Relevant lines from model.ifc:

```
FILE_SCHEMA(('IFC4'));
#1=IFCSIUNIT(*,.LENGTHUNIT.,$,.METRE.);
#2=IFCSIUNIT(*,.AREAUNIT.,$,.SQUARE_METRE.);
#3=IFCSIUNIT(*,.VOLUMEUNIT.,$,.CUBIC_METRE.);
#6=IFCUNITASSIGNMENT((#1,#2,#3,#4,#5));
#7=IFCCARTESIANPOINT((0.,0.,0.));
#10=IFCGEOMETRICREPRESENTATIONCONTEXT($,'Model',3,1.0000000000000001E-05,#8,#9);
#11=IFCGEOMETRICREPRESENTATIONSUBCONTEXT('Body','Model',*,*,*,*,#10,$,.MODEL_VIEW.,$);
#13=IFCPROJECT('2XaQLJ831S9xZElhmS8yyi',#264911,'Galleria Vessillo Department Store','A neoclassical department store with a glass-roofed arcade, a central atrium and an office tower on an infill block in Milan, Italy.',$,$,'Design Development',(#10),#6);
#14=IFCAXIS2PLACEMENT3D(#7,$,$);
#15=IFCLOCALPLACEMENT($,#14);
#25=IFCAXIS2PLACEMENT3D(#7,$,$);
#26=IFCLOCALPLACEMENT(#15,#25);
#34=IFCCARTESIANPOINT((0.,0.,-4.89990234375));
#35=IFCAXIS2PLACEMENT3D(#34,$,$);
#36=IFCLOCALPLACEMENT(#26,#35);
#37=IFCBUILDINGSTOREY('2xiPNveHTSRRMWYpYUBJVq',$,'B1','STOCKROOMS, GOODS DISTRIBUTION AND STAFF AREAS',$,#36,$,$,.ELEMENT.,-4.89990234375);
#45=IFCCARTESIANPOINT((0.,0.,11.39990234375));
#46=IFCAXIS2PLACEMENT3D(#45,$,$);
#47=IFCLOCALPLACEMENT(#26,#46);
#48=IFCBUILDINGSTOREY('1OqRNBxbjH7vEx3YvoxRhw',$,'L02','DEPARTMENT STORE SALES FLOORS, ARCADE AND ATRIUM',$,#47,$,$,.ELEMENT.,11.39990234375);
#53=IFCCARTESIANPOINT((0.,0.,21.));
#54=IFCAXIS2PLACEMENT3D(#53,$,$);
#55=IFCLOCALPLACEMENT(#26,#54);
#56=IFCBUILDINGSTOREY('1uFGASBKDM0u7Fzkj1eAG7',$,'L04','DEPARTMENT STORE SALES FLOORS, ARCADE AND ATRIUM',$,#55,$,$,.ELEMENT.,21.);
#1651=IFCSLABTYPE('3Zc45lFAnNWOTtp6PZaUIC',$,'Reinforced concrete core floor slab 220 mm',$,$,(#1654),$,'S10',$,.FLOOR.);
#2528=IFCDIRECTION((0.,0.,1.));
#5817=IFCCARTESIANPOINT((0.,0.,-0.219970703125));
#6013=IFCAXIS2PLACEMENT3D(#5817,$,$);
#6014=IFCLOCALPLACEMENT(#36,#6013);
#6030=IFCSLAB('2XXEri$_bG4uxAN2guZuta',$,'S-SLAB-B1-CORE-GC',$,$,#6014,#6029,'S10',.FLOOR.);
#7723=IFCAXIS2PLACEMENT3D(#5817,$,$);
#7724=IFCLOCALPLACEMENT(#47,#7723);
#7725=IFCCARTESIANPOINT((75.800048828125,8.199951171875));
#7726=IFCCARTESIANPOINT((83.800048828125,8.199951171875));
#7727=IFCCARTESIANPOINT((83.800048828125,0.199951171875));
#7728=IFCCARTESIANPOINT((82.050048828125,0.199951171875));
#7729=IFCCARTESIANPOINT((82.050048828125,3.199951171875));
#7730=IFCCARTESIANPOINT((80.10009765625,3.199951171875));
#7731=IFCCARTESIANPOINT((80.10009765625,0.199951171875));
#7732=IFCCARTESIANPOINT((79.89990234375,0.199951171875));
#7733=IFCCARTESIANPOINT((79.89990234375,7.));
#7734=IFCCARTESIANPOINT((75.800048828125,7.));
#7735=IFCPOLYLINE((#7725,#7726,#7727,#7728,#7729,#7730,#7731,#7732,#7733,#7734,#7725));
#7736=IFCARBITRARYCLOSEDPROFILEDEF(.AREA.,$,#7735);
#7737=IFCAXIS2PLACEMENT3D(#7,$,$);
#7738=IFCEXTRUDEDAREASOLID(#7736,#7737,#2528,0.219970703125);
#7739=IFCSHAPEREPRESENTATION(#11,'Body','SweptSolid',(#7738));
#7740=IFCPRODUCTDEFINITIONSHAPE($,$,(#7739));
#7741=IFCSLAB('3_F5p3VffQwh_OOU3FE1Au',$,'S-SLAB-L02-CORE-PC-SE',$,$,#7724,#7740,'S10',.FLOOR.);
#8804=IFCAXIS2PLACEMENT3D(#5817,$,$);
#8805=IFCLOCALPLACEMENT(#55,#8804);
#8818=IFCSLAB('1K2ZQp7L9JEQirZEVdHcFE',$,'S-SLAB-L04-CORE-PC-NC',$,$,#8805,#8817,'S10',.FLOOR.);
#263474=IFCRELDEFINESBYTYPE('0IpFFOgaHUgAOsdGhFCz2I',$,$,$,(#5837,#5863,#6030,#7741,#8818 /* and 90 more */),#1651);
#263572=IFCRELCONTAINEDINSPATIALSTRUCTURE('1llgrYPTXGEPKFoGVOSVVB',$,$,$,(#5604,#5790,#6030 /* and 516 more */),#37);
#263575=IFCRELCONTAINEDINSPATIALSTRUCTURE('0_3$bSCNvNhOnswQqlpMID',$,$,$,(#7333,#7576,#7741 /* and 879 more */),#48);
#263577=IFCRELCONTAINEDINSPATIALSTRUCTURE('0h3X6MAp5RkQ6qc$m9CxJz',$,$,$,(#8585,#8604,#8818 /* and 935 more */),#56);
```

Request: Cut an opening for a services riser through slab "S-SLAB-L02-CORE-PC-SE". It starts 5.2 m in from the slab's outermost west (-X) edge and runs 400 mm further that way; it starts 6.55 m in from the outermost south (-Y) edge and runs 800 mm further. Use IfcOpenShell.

```python
import numpy as np
import ifcopenshell
import ifcopenshell.api.feature
import ifcopenshell.api.geometry
import ifcopenshell.api.root
import ifcopenshell.geom
import ifcopenshell.util.placement
import ifcopenshell.util.representation
import ifcopenshell.util.shape
import ifcopenshell.util.unit

model = ifcopenshell.open("model.ifc")
unit_scale = ifcopenshell.util.unit.calculate_unit_scale(model)
settings = ifcopenshell.geom.settings()


def volume(element):
    """Net volume in cubic metres, openings subtracted."""
    shape = ifcopenshell.geom.create_shape(settings, element)
    return ifcopenshell.util.shape.get_volume(shape.geometry)


slab = model.by_guid("3_F5p3VffQwh_OOU3FE1Au")
before = volume(slab)

# Extent in the slab's own axes, in metres. The edges named are its -X and -Y sides.
slab_shape = ifcopenshell.geom.create_shape(settings, slab)
vertices = ifcopenshell.util.shape.get_vertices(slab_shape.geometry)
x_min, y_min, bottom = vertices.min(axis=0)
top = vertices[:, 2].max()

opening = ifcopenshell.api.root.create_entity(model, ifc_class="IfcOpeningElement", name="Services riser opening", predefined_type="OPENING")
context = ifcopenshell.util.representation.get_context(model, "Model", "Body", "MODEL_VIEW")
width, depth = 0.4, 0.8
outline = [(0.0, 0.0), (width, 0.0), (width, depth), (0.0, depth), (0.0, 0.0)]
# Overshoot both faces by 50 mm so the cut is clean.
shape = ifcopenshell.api.geometry.add_slab_representation(
    model, context=context, depth=top - bottom + 0.1, polyline=outline
)
ifcopenshell.api.geometry.assign_representation(model, product=opening, representation=shape)

matrix = ifcopenshell.util.placement.get_local_placement(slab.ObjectPlacement)
matrix[:, 3] = matrix @ np.append(np.array([x_min + 5.2, y_min + 6.55, bottom - 0.05]) / unit_scale, 1.0)
ifcopenshell.api.geometry.edit_object_placement(model, product=opening, matrix=matrix, is_si=False)
ifcopenshell.api.feature.add_feature(model, feature=opening, element=slab)

after = volume(slab)

print(f"slab volume {before:.3f} -> {after:.3f} m3")

model.write("model_rev.ifc")
```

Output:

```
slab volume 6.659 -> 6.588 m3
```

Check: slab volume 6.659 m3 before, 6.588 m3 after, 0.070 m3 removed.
